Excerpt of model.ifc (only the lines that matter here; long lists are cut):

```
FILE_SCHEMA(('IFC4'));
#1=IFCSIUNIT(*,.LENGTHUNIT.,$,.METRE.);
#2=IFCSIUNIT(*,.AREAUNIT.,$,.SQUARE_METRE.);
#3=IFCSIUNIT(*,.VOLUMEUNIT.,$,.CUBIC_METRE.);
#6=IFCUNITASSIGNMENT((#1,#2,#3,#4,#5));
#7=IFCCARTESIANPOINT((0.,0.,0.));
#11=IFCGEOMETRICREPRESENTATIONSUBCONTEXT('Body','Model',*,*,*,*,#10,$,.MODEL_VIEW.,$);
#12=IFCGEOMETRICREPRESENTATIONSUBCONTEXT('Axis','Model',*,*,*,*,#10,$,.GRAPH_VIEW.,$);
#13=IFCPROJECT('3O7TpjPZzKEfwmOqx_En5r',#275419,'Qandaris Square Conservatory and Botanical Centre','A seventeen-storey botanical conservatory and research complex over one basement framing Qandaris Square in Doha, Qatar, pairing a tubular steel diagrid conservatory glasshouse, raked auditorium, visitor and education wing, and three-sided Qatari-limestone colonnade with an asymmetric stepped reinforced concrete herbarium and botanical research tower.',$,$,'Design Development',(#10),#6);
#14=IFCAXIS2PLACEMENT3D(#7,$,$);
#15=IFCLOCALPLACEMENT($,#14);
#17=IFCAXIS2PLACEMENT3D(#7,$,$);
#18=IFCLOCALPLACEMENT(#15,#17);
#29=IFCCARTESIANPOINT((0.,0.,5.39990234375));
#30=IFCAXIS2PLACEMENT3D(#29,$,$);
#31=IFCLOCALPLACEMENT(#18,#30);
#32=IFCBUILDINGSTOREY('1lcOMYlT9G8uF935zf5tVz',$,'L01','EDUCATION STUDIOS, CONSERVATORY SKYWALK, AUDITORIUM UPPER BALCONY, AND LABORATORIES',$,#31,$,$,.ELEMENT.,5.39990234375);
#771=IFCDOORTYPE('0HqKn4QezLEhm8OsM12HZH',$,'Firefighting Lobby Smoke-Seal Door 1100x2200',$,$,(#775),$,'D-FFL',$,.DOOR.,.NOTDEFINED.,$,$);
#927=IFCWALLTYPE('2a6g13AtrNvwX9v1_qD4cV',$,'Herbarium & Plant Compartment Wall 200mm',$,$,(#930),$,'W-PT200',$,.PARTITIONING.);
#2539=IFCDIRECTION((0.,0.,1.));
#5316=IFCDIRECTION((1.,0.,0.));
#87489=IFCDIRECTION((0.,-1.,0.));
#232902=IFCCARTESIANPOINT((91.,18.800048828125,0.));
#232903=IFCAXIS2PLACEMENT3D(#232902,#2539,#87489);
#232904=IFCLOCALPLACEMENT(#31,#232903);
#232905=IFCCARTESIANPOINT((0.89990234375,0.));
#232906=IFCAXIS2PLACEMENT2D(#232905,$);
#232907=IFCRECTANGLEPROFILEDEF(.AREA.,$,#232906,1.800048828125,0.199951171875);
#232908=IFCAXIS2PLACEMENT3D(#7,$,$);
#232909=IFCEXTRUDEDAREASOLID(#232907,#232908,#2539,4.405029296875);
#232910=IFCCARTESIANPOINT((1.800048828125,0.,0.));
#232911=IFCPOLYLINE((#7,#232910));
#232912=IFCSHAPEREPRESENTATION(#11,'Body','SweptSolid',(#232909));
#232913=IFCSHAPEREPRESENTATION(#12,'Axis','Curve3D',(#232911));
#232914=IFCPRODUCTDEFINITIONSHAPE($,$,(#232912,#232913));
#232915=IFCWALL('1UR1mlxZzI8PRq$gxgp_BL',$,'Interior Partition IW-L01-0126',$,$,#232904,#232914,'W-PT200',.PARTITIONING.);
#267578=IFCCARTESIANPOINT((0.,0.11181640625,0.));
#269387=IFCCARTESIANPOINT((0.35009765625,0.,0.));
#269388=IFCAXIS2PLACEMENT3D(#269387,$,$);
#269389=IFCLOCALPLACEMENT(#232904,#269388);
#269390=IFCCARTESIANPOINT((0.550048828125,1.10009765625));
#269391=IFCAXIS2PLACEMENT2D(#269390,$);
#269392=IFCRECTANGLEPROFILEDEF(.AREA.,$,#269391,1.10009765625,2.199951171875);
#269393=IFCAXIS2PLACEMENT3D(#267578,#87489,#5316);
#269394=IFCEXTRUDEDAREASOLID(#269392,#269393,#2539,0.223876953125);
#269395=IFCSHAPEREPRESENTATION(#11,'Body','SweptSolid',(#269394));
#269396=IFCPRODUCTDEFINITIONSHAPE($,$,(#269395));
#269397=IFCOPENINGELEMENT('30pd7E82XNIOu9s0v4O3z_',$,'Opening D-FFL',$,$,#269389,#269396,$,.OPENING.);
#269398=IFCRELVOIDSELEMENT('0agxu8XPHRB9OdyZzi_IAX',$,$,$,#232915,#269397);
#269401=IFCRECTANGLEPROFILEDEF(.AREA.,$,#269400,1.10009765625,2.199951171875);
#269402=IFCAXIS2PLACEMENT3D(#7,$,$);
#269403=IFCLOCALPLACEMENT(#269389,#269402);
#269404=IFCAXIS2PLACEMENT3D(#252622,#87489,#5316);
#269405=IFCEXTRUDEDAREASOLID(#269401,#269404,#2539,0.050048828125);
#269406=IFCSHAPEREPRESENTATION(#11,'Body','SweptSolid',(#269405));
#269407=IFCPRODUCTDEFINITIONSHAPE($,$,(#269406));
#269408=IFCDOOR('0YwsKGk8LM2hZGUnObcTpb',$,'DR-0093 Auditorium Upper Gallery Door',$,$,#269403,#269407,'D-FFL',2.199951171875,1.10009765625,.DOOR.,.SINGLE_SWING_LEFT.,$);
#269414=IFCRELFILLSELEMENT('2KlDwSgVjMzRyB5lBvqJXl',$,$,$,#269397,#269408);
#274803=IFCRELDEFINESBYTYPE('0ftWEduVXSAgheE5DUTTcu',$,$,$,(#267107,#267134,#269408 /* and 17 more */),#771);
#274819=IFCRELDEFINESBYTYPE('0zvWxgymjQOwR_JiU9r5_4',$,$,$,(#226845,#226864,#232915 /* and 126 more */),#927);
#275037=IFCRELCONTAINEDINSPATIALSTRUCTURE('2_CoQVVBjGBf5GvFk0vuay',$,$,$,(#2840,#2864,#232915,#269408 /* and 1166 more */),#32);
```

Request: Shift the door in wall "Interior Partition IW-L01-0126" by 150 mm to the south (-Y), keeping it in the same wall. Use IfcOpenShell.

```python
import ifcopenshell
import ifcopenshell.api.geometry
import ifcopenshell.util.placement

model = ifcopenshell.open("model.ifc")

door = model.by_guid("0YwsKGk8LM2hZGUnObcTpb")
opening = door.FillsVoids[0].RelatingOpeningElement
wall = opening.VoidsElements[0].RelatingBuildingElement

wall_matrix = ifcopenshell.util.placement.get_local_placement(wall.ObjectPlacement)
shift = wall_matrix[:3, 0] * 0.15
before = ifcopenshell.util.placement.get_local_placement(door.ObjectPlacement)[:3, 3].copy()

# The door is placed relative to its opening, so it follows when the opening moves.
matrix = ifcopenshell.util.placement.get_local_placement(opening.ObjectPlacement)
matrix[:3, 3] += shift
ifcopenshell.api.geometry.edit_object_placement(
    model, product=opening, matrix=matrix, is_si=False, should_transform_children=True
)

after = ifcopenshell.util.placement.get_local_placement(door.ObjectPlacement)[:3, 3]
print("door moved by", (after - before).round(3) + 0.0)

model.write("model_v2.ifc")
```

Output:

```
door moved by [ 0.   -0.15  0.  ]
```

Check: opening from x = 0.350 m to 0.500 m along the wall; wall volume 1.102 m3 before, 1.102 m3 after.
